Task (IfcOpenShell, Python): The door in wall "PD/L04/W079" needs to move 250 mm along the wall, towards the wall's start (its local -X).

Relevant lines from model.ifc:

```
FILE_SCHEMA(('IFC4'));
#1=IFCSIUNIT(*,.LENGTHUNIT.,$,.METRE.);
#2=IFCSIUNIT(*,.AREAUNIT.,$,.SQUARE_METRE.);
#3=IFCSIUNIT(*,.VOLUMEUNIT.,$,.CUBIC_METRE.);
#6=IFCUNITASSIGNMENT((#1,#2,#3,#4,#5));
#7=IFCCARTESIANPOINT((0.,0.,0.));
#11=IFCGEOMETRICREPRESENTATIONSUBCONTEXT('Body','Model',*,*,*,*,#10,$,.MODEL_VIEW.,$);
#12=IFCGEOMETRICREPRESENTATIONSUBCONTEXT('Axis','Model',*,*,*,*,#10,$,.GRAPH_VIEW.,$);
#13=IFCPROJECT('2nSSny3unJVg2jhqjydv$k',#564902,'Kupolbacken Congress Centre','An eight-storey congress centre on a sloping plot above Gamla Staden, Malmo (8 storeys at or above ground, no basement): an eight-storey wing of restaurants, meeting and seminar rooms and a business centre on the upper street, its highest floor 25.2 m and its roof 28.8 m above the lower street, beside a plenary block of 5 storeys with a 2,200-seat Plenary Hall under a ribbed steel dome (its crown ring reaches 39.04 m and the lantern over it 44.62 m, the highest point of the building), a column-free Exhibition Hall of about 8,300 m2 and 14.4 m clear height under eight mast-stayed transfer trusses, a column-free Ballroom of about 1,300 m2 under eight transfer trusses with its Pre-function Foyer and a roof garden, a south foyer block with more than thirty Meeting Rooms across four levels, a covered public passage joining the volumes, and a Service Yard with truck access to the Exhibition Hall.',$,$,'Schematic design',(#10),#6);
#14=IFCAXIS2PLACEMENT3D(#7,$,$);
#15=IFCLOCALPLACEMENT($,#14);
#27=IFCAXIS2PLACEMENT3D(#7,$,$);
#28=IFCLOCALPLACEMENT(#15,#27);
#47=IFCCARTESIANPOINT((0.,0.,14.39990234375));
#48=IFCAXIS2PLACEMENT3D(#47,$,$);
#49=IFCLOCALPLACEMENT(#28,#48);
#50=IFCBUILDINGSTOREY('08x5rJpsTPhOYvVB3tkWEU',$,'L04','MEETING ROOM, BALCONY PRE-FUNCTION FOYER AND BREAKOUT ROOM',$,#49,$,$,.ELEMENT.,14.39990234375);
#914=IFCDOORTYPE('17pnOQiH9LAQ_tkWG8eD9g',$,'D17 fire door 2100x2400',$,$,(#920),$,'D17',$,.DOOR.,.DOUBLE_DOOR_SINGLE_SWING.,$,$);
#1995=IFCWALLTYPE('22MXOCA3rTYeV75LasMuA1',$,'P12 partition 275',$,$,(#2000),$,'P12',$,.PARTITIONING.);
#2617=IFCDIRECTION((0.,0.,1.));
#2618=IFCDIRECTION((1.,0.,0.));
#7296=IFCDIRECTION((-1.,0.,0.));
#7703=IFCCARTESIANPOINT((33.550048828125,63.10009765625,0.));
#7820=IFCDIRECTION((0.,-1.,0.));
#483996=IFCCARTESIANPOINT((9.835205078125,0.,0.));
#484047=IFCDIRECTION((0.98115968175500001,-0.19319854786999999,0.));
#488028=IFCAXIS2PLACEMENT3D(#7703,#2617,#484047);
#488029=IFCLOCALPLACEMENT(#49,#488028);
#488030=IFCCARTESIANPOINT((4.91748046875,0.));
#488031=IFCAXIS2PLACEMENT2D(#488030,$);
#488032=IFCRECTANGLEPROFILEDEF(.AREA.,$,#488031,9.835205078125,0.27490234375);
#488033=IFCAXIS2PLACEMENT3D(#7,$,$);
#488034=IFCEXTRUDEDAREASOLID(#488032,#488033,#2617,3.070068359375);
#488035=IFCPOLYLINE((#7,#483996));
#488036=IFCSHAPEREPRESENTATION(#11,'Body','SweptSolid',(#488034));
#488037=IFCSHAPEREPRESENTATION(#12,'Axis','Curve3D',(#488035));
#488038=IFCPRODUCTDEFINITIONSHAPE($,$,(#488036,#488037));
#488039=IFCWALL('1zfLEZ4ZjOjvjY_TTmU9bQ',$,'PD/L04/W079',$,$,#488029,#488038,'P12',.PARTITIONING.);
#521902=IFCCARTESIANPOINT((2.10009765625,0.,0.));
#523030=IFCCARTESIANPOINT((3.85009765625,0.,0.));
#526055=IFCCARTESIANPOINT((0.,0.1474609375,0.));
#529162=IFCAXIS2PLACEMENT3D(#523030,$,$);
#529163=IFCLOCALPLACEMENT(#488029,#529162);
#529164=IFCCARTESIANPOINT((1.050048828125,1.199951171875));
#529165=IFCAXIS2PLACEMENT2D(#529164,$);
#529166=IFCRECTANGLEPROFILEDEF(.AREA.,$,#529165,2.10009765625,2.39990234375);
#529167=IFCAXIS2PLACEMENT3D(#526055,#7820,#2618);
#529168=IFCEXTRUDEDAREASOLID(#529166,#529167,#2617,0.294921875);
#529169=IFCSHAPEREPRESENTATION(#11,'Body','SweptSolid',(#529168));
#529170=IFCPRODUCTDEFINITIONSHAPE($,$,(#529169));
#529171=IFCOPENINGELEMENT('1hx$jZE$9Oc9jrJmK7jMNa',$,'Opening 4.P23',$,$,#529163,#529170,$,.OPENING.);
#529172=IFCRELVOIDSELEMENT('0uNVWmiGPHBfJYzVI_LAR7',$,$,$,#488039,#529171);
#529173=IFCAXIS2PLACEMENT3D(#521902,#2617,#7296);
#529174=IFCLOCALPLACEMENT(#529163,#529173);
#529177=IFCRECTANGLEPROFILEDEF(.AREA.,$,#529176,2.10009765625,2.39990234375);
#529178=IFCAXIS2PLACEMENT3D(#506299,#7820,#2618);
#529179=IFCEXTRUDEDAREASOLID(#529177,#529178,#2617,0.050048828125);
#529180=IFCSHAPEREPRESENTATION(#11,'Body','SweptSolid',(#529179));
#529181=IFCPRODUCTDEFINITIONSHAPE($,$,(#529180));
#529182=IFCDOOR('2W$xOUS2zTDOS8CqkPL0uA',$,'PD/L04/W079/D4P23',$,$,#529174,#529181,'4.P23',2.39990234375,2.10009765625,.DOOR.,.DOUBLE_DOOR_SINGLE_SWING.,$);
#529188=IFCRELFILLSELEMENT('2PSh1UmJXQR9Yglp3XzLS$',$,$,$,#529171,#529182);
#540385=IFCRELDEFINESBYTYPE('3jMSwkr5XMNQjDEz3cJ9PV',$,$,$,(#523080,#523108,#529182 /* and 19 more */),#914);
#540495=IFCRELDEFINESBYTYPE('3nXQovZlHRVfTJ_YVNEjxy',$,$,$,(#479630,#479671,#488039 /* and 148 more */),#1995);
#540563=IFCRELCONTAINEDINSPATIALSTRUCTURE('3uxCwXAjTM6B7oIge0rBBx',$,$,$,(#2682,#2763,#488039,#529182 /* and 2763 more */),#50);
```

```python
import ifcopenshell
import ifcopenshell.api.geometry
import ifcopenshell.util.placement
import ifcopenshell.util.unit

model = ifcopenshell.open("model.ifc")
unit_scale = ifcopenshell.util.unit.calculate_unit_scale(model)

door = model.by_guid("2W$xOUS2zTDOS8CqkPL0uA")
opening = door.FillsVoids[0].RelatingOpeningElement
wall = opening.VoidsElements[0].RelatingBuildingElement

wall_matrix = ifcopenshell.util.placement.get_local_placement(wall.ObjectPlacement)
shift = wall_matrix[:3, 0] * -0.25 / unit_scale
before = ifcopenshell.util.placement.get_local_placement(door.ObjectPlacement)[:3, 3].copy()

# The door is placed relative to its opening, so it follows when the opening moves.
matrix = ifcopenshell.util.placement.get_local_placement(opening.ObjectPlacement)
matrix[:3, 3] += shift
ifcopenshell.api.geometry.edit_object_placement(
    model, product=opening, matrix=matrix, is_si=False, should_transform_children=True
)

after = ifcopenshell.util.placement.get_local_placement(door.ObjectPlacement)[:3, 3]
print("door moved by", (after - before).round(3) + 0.0)

model.write("model_edited.ifc")
```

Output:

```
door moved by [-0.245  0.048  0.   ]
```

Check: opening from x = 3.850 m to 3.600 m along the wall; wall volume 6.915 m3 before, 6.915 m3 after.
